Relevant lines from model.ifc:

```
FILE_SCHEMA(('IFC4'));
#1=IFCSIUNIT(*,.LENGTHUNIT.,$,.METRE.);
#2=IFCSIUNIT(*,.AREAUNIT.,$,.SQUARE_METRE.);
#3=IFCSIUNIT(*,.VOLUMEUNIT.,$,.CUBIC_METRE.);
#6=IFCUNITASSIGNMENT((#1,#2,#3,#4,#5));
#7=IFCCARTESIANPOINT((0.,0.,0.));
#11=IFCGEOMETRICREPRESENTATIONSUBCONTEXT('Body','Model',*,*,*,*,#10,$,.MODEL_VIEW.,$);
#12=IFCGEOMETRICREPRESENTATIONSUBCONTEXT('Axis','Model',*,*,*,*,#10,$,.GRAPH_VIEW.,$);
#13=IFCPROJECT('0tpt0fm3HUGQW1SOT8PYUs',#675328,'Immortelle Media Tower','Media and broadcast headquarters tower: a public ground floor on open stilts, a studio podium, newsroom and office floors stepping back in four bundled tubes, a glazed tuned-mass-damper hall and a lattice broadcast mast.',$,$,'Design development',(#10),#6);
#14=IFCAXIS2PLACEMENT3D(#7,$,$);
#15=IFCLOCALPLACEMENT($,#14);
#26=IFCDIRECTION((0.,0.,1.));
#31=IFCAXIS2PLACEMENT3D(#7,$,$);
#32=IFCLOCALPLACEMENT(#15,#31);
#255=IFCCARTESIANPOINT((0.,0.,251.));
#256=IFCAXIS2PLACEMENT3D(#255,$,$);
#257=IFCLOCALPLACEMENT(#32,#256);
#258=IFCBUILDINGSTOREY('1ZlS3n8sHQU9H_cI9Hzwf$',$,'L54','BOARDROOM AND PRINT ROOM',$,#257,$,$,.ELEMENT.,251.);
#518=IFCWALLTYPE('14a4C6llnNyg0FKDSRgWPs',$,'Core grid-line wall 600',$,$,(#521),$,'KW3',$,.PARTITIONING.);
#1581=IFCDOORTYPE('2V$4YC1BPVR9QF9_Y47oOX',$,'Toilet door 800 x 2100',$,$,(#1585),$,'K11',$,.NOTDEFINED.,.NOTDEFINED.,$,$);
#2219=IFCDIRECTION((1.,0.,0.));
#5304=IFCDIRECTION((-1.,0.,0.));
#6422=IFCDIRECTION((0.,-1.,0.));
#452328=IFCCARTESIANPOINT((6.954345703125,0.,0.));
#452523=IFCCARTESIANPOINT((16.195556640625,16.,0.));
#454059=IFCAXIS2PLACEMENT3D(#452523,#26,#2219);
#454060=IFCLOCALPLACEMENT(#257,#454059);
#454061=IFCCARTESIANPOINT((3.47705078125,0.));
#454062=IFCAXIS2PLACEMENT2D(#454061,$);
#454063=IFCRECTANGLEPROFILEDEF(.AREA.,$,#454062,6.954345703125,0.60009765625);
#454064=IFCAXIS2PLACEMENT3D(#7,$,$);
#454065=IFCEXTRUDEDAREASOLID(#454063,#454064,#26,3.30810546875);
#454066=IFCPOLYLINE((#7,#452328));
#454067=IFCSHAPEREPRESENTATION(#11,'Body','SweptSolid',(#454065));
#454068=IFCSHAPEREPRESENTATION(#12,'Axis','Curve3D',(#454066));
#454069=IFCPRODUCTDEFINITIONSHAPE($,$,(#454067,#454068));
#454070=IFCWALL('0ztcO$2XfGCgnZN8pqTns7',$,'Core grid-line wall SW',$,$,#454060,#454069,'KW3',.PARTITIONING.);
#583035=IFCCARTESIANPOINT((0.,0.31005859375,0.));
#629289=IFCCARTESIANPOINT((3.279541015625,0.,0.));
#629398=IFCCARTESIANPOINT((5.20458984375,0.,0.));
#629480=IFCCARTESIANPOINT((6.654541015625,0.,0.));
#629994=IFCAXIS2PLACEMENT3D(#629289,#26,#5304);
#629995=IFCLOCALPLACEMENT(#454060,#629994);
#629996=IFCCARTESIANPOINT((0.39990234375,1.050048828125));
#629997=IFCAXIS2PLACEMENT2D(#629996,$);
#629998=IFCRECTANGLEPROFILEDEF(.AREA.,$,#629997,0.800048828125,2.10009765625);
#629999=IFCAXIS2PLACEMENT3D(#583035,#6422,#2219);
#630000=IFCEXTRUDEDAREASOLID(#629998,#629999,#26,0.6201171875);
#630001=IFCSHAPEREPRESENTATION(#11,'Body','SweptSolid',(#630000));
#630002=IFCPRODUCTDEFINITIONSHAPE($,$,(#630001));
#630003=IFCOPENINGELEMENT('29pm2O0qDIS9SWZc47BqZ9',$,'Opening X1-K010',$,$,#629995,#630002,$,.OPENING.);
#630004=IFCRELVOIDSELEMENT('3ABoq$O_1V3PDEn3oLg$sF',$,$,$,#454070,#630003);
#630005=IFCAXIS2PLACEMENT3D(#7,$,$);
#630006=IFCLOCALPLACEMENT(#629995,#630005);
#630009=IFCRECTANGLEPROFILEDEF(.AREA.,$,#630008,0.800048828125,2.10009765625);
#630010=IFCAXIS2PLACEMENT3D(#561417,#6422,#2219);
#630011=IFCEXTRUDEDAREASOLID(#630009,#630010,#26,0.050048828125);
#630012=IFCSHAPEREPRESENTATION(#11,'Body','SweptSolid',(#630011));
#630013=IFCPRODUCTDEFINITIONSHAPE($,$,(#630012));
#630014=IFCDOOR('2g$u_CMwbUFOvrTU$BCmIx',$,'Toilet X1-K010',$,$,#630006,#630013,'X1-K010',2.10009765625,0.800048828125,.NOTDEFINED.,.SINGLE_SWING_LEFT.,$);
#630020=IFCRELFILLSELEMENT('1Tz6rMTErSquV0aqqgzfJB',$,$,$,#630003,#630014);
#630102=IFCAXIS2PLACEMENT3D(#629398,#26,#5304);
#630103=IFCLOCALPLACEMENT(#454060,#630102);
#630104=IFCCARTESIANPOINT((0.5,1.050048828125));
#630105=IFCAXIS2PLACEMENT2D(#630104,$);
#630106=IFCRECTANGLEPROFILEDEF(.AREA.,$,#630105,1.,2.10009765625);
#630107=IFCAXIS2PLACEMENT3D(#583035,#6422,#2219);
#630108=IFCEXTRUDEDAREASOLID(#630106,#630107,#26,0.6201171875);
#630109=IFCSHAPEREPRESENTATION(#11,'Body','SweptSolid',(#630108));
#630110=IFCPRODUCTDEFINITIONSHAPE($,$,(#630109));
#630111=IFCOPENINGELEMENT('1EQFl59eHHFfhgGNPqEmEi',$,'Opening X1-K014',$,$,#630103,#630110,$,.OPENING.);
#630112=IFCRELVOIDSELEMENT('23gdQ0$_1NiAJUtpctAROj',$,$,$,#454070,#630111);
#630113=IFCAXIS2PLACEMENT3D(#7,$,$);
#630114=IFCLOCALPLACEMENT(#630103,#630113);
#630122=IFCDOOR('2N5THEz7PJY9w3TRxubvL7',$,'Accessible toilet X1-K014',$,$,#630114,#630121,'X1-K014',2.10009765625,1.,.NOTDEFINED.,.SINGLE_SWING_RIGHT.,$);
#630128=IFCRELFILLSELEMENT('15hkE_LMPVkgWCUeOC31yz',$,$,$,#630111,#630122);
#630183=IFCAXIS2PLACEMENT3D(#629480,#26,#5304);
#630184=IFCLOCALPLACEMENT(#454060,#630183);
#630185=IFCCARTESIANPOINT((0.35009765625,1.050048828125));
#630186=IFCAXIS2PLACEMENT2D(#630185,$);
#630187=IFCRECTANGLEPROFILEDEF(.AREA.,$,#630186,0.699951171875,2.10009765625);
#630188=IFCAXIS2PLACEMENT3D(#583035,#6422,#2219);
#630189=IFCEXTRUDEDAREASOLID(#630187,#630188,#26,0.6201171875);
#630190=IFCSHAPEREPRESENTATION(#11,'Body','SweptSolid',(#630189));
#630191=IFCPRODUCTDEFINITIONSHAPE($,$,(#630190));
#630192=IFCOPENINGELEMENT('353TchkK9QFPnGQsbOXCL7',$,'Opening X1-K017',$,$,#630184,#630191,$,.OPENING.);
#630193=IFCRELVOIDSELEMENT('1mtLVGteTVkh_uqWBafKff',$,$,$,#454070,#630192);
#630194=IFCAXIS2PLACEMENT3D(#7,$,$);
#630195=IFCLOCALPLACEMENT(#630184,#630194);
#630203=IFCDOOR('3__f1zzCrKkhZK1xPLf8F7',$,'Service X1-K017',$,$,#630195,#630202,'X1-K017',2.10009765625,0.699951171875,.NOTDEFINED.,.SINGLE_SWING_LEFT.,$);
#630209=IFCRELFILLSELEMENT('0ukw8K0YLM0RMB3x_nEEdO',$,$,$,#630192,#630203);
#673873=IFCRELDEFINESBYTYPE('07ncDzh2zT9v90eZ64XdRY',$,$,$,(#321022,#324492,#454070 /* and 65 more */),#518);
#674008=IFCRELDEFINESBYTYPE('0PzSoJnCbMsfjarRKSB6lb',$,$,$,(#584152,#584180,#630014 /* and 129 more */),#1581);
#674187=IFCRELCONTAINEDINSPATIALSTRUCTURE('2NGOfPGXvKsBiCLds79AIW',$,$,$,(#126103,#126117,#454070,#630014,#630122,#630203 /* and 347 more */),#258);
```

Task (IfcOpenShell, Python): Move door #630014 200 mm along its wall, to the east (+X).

```python
import ifcopenshell
import ifcopenshell.api.geometry
import ifcopenshell.util.placement

model = ifcopenshell.open("model.ifc")

door = model.by_guid("2g$u_CMwbUFOvrTU$BCmIx")
opening = door.FillsVoids[0].RelatingOpeningElement
wall = opening.VoidsElements[0].RelatingBuildingElement

wall_matrix = ifcopenshell.util.placement.get_local_placement(wall.ObjectPlacement)
shift = wall_matrix[:3, 0] * 0.2
before = ifcopenshell.util.placement.get_local_placement(door.ObjectPlacement)[:3, 3].copy()

# The door is placed relative to its opening, so it follows when the opening moves.
matrix = ifcopenshell.util.placement.get_local_placement(opening.ObjectPlacement)
matrix[:3, 3] += shift
ifcopenshell.api.geometry.edit_object_placement(
    model, product=opening, matrix=matrix, is_si=False, should_transform_children=True
)

after = ifcopenshell.util.placement.get_local_placement(door.ObjectPlacement)[:3, 3]
print("door moved by", (after - before).round(3) + 0.0)

model.write("model_v2.ifc")
```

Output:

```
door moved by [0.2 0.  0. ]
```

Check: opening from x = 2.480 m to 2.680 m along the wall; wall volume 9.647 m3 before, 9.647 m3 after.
